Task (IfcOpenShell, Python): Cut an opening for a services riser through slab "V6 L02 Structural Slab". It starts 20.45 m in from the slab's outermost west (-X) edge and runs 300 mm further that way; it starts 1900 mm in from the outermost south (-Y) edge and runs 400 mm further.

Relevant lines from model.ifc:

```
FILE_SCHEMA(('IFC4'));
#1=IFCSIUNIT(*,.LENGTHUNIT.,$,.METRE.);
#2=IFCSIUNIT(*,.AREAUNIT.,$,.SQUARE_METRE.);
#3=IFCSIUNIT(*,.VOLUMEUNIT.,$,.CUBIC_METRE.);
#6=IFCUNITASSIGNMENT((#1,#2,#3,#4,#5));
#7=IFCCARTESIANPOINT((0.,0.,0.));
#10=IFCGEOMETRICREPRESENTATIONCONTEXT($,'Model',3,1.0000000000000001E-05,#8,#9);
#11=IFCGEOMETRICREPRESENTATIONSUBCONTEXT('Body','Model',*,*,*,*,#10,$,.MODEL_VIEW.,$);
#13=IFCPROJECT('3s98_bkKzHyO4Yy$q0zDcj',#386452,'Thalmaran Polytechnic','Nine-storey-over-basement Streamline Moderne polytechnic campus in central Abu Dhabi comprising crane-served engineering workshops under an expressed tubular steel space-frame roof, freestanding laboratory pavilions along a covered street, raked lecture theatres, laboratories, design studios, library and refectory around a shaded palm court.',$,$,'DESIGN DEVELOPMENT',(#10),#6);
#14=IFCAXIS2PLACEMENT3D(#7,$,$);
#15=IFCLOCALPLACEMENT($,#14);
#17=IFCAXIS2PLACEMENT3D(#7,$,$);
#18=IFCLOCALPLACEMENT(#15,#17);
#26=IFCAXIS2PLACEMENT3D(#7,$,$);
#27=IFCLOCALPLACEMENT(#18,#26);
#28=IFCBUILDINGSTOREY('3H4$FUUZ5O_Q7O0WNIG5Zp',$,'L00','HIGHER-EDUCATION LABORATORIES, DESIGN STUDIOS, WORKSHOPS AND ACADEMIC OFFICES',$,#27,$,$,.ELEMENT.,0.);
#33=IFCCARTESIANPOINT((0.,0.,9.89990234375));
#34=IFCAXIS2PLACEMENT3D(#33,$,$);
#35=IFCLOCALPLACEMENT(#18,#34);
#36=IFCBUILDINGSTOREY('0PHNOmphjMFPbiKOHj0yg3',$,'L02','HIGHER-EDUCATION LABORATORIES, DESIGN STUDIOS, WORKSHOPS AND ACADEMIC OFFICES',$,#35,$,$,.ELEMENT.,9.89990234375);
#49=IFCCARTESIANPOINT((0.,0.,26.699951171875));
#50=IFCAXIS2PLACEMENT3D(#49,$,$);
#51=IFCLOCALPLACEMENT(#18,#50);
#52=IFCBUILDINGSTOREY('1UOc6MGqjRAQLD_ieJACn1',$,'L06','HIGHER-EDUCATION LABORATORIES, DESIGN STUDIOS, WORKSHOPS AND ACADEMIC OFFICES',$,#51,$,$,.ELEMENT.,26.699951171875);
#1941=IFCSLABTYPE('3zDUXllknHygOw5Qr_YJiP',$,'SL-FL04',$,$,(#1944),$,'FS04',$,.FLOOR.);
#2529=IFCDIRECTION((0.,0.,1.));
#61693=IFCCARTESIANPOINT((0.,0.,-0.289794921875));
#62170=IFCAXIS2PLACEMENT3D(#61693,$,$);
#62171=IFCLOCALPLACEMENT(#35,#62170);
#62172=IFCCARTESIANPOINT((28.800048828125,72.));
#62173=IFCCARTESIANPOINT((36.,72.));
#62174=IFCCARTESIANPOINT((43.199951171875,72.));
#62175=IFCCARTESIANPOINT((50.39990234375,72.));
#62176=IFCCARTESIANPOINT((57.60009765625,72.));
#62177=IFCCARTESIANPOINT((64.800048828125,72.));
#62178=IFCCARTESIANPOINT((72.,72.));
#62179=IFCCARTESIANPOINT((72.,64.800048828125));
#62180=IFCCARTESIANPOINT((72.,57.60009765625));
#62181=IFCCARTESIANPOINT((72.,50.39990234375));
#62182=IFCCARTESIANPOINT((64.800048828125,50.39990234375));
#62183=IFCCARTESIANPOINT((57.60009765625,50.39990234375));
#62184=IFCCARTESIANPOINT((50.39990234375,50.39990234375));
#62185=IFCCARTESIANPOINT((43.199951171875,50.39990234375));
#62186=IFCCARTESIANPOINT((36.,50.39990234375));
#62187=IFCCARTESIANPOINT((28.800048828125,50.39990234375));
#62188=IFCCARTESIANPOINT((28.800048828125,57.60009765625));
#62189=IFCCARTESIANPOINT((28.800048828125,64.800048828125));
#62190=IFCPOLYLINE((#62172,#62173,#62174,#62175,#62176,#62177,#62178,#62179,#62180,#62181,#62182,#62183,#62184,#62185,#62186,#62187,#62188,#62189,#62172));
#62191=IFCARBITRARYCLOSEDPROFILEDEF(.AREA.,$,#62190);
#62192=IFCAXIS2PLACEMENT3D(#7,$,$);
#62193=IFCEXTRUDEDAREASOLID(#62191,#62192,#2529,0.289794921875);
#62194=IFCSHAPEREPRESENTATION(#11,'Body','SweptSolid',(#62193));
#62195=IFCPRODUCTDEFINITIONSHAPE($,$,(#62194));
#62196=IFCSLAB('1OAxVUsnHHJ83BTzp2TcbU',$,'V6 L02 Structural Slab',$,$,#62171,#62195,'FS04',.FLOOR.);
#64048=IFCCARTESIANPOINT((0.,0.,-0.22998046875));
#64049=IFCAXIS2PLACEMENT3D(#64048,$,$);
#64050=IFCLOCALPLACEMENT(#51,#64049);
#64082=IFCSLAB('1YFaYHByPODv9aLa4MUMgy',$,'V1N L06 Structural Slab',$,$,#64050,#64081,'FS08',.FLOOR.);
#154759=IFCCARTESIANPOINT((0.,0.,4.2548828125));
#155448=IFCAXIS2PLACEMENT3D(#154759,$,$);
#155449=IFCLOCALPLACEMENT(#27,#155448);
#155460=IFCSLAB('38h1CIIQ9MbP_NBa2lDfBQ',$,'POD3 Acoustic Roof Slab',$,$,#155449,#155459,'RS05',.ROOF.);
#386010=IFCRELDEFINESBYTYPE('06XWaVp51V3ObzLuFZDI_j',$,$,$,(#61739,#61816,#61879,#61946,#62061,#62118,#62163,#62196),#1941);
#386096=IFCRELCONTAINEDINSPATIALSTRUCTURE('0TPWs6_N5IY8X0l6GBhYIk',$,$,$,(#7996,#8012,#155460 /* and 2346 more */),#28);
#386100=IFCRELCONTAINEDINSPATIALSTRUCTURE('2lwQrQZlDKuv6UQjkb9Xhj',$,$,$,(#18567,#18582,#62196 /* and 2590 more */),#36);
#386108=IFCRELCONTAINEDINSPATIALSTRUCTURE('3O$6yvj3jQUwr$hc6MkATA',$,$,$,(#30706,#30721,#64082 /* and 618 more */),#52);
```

```python
import numpy as np
import ifcopenshell
import ifcopenshell.api.feature
import ifcopenshell.api.geometry
import ifcopenshell.api.root
import ifcopenshell.geom
import ifcopenshell.util.placement
import ifcopenshell.util.representation
import ifcopenshell.util.shape
import ifcopenshell.util.unit

model = ifcopenshell.open("model.ifc")
unit_scale = ifcopenshell.util.unit.calculate_unit_scale(model)
settings = ifcopenshell.geom.settings()


def volume(element):
    """Net volume in cubic metres, openings subtracted."""
    shape = ifcopenshell.geom.create_shape(settings, element)
    return ifcopenshell.util.shape.get_volume(shape.geometry)


slab = model.by_guid("1OAxVUsnHHJ83BTzp2TcbU")
before = volume(slab)

# Extent in the slab's own axes, in metres. The edges named are its -X and -Y sides.
slab_shape = ifcopenshell.geom.create_shape(settings, slab)
vertices = ifcopenshell.util.shape.get_vertices(slab_shape.geometry)
x_min, y_min, bottom = vertices.min(axis=0)
top = vertices[:, 2].max()

opening = ifcopenshell.api.root.create_entity(model, ifc_class="IfcOpeningElement", name="Services riser opening", predefined_type="OPENING")
context = ifcopenshell.util.representation.get_context(model, "Model", "Body", "MODEL_VIEW")
width, depth = 0.3, 0.4
outline = [(0.0, 0.0), (width, 0.0), (width, depth), (0.0, depth), (0.0, 0.0)]
# Overshoot both faces by 50 mm so the cut is clean.
shape = ifcopenshell.api.geometry.add_slab_representation(
    model, context=context, depth=top - bottom + 0.1, polyline=outline
)
ifcopenshell.api.geometry.assign_representation(model, product=opening, representation=shape)

matrix = ifcopenshell.util.placement.get_local_placement(slab.ObjectPlacement)
matrix[:, 3] = matrix @ np.append(np.array([x_min + 20.45, y_min + 1.9, bottom - 0.05]) / unit_scale, 1.0)
ifcopenshell.api.geometry.edit_object_placement(model, product=opening, matrix=matrix, is_si=False)
ifcopenshell.api.feature.add_feature(model, feature=opening, element=slab)

after = volume(slab)

print(f"slab volume {before:.3f} -> {after:.3f} m3")

model.write("model_edited.ifc")
```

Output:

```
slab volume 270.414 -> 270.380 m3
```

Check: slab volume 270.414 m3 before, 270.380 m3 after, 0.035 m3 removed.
